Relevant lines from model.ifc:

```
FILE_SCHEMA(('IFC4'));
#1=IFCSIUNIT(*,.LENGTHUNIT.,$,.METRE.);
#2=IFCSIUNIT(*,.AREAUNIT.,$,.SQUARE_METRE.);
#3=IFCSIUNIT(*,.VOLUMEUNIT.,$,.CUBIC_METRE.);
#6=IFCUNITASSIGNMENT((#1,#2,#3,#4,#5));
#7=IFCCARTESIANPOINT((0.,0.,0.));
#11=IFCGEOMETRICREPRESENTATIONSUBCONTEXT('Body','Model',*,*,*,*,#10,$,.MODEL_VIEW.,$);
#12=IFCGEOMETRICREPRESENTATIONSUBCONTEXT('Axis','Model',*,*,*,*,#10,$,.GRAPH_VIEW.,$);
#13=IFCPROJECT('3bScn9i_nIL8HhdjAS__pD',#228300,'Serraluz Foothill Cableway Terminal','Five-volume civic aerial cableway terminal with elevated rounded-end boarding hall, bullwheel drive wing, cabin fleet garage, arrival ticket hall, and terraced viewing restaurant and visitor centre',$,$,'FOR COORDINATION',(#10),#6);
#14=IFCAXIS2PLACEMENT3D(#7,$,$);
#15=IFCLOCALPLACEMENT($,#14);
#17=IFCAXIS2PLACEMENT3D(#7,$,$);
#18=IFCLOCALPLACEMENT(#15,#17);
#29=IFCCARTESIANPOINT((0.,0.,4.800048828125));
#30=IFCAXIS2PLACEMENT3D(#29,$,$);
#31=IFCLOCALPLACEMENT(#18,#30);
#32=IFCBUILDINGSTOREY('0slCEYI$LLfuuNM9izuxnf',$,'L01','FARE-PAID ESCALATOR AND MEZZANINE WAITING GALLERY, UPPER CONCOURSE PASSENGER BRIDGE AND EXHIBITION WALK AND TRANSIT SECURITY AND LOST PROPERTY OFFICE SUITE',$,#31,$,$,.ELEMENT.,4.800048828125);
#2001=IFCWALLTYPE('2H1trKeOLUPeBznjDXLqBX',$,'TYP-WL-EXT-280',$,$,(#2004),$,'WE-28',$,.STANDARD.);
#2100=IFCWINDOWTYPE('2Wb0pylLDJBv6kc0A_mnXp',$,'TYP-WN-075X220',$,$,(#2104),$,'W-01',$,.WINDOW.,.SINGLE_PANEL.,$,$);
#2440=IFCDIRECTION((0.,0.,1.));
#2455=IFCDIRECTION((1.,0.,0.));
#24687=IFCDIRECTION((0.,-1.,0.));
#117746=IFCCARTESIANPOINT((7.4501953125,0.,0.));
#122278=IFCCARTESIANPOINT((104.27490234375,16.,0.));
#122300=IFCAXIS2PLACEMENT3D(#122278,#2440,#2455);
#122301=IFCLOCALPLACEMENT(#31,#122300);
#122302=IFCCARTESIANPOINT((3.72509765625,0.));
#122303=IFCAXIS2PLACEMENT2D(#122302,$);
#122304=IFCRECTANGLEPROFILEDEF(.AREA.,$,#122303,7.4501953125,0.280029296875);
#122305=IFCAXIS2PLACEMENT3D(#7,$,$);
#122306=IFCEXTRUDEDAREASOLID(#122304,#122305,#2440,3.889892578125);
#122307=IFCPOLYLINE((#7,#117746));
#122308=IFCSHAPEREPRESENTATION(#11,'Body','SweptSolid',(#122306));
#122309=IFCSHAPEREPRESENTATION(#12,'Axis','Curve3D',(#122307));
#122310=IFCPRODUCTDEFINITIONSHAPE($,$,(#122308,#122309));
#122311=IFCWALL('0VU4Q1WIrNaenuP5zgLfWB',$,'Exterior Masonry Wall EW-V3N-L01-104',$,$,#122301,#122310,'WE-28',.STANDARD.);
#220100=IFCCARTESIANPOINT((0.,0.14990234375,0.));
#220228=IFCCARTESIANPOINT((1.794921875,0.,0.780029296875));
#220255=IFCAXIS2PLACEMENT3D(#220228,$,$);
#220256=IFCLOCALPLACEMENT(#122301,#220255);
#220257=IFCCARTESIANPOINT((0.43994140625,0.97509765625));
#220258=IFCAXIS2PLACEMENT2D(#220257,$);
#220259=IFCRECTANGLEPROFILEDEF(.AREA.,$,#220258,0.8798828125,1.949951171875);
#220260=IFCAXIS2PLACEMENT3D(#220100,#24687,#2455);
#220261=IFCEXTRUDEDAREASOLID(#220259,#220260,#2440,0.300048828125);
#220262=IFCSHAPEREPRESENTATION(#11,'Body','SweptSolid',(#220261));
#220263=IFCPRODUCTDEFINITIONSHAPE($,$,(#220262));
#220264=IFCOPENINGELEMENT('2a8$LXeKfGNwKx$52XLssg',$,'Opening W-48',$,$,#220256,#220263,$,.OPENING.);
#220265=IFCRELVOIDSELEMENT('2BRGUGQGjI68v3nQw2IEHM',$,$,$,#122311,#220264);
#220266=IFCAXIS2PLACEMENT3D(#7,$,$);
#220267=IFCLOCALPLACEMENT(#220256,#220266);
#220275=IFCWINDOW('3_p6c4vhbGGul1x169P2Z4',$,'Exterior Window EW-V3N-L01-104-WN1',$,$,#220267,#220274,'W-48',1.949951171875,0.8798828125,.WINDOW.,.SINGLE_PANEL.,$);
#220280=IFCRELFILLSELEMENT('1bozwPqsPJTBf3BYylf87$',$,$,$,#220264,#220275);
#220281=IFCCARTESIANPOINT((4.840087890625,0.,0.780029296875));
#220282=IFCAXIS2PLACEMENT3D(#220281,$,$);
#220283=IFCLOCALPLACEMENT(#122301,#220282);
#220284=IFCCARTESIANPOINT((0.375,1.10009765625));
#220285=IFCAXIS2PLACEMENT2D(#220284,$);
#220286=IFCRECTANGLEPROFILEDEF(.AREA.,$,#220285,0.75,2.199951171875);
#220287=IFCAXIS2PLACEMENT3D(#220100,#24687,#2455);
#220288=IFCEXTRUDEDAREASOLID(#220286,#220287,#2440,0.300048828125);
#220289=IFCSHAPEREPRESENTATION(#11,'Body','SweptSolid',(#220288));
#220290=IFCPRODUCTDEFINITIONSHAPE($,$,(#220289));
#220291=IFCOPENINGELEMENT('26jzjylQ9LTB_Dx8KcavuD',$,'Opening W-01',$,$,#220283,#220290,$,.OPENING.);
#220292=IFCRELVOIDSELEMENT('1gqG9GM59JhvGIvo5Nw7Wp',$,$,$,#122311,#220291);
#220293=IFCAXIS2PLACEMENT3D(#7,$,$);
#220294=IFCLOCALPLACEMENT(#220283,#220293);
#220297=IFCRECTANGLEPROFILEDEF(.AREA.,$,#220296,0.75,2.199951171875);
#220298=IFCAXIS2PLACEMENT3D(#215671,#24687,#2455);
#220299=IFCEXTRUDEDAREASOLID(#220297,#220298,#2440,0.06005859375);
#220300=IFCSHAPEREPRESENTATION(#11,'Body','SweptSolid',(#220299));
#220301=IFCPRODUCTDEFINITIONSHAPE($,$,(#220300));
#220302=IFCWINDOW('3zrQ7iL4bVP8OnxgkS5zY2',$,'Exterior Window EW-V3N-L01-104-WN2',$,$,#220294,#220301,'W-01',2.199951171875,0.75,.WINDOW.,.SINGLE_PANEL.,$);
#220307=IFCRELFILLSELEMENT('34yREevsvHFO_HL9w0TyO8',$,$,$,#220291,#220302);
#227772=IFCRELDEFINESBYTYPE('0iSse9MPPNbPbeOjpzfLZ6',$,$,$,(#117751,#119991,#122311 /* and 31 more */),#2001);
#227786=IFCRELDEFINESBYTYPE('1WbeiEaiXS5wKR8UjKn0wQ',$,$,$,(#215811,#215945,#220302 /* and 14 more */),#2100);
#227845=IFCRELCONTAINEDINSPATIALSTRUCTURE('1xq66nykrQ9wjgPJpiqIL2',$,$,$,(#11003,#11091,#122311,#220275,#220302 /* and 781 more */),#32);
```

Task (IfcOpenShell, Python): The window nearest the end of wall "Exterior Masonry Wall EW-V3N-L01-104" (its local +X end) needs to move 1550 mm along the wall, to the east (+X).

```python
import ifcopenshell
import ifcopenshell.api.geometry
import ifcopenshell.util.placement
import ifcopenshell.util.unit

model = ifcopenshell.open("model.ifc")
unit_scale = ifcopenshell.util.unit.calculate_unit_scale(model)

window = model.by_guid("3zrQ7iL4bVP8OnxgkS5zY2")
opening = window.FillsVoids[0].RelatingOpeningElement
wall = opening.VoidsElements[0].RelatingBuildingElement

wall_matrix = ifcopenshell.util.placement.get_local_placement(wall.ObjectPlacement)
shift = wall_matrix[:3, 0] * 1.55 / unit_scale
before = ifcopenshell.util.placement.get_local_placement(window.ObjectPlacement)[:3, 3].copy()

# The window is placed relative to its opening, so it follows when the opening moves.
matrix = ifcopenshell.util.placement.get_local_placement(opening.ObjectPlacement)
matrix[:3, 3] += shift
ifcopenshell.api.geometry.edit_object_placement(
    model, product=opening, matrix=matrix, is_si=False, should_transform_children=True
)

after = ifcopenshell.util.placement.get_local_placement(window.ObjectPlacement)[:3, 3]
print("window moved by", (after - before).round(3) + 0.0)

model.write("model-out.ifc")
```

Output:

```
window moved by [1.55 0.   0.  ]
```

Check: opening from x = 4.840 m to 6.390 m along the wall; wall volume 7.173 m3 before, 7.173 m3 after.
